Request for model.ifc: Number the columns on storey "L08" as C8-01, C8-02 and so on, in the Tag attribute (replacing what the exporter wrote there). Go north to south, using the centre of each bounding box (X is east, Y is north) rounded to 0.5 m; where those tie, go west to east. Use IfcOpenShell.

First a look at what the model holds.

```python
import ifcopenshell
import ifcopenshell.util.element
import ifcopenshell.util.placement

model = ifcopenshell.open("model.ifc")
print(model.schema)
storey = next(s for s in model.by_type("IfcBuildingStorey") if s.Name == "L08")
columns = [e for e in ifcopenshell.util.element.get_decomposition(storey) if e.is_a("IfcColumn")]
for e in sorted(columns, key=lambda e: e.id()):
    origin = ifcopenshell.util.placement.get_local_placement(e.ObjectPlacement)[:3, 3]
    print(e.id(), e.Tag, e.Name, origin.round(2) + 0.0, sep=" | ")
```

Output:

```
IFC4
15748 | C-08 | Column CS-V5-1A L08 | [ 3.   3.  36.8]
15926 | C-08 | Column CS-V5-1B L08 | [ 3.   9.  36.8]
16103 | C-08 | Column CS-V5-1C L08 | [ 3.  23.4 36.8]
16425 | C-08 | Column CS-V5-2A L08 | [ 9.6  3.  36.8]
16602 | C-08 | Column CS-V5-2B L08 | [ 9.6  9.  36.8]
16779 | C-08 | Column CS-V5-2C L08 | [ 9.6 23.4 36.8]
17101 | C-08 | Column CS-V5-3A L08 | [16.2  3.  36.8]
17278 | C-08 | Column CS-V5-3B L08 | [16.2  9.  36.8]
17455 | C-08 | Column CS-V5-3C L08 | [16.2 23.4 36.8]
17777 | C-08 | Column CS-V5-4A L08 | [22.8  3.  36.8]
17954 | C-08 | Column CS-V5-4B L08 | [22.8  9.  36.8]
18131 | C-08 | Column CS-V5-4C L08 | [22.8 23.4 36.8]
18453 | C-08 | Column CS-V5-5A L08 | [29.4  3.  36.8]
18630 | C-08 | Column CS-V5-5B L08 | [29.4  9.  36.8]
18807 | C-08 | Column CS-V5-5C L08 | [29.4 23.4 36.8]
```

```python
import ifcopenshell
import ifcopenshell.geom
import ifcopenshell.util.element
import ifcopenshell.util.shape

model = ifcopenshell.open("model.ifc")
settings = ifcopenshell.geom.settings()
settings.set("use-world-coords", True)


def centre(element):
    shape = ifcopenshell.geom.create_shape(settings, element)
    return ifcopenshell.util.shape.get_bbox_centroid(shape.geometry)


storey = next(s for s in model.by_type("IfcBuildingStorey") if s.Name == "L08")
columns = [e for e in ifcopenshell.util.element.get_decomposition(storey) if e.is_a("IfcColumn")]

# Insertion points can sit at a corner or the storey origin, so sort by the geometry (in metres).
centres = {e: centre(e) for e in columns}
columns.sort(key=lambda e: (-round(centres[e][1] / 0.5), centres[e][0]))

for i, e in enumerate(columns, start=1):
    number = f"C8-{i:02d}"
    e.Tag = number
    print(e.id(), number)

model.write("model_v2.ifc")
```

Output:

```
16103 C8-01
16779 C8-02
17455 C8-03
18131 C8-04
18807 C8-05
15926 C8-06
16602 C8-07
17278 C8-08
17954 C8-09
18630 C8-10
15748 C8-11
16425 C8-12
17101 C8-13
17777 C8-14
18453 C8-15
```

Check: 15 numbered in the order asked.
